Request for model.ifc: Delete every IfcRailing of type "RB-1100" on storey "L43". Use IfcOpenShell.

First a look at what the model holds.

```python
import ifcopenshell
import ifcopenshell.util.element

model = ifcopenshell.open("model.ifc")
print(model.schema)
storey = next(s for s in model.by_type("IfcBuildingStorey") if s.Name == "L43")
railings = [e for e in ifcopenshell.util.element.get_decomposition(storey) if e.is_a("IfcRailing")]
seen = {}
for e in railings:
    element_type = ifcopenshell.util.element.get_type(e)
    name = element_type.Name if element_type not in (None, e) else None
    seen[name] = seen.get(name, 0) + 1
for name, count in sorted(seen.items(), key=str):
    print(count, "x", name)
```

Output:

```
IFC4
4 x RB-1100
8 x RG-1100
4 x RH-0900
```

```python
import ifcopenshell
import ifcopenshell.api.root
import ifcopenshell.util.element

model = ifcopenshell.open("model.ifc")

storey = next(s for s in model.by_type("IfcBuildingStorey") if s.Name == "L43")
railings = [e for e in ifcopenshell.util.element.get_decomposition(storey) if e.is_a("IfcRailing")]
targets = [e for e in railings if (t := ifcopenshell.util.element.get_type(e)) not in (None, e) and t.Name == "RB-1100"]

for e in targets:
    ifcopenshell.api.root.remove_product(model, product=e)
print(len(targets), "removed")

model.write("model_v2.ifc")
```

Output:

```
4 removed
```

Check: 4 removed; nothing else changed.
